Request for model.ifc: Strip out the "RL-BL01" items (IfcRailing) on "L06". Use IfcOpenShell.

First a look at what the model holds.

```python
import ifcopenshell
import ifcopenshell.util.element

model = ifcopenshell.open("model.ifc")
print(model.schema)
storey = next(s for s in model.by_type("IfcBuildingStorey") if s.Name == "L06")
railings = [e for e in ifcopenshell.util.element.get_decomposition(storey) if e.is_a("IfcRailing")]
seen = {}
for e in railings:
    element_type = ifcopenshell.util.element.get_type(e)
    name = element_type.Name if element_type not in (None, e) else None
    seen[name] = seen.get(name, 0) + 1
for name, count in sorted(seen.items(), key=str):
    print(count, "x", name)
```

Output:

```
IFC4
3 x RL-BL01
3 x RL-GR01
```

```python
import ifcopenshell
import ifcopenshell.api.root
import ifcopenshell.util.element

model = ifcopenshell.open("model.ifc")

storey = next(s for s in model.by_type("IfcBuildingStorey") if s.Name == "L06")
railings = [e for e in ifcopenshell.util.element.get_decomposition(storey) if e.is_a("IfcRailing")]
targets = [e for e in railings if (t := ifcopenshell.util.element.get_type(e)) not in (None, e) and t.Name == "RL-BL01"]

for e in targets:
    ifcopenshell.api.root.remove_product(model, product=e)
print(len(targets), "removed")

model.write("model_rev.ifc")
```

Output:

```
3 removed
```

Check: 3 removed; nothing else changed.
